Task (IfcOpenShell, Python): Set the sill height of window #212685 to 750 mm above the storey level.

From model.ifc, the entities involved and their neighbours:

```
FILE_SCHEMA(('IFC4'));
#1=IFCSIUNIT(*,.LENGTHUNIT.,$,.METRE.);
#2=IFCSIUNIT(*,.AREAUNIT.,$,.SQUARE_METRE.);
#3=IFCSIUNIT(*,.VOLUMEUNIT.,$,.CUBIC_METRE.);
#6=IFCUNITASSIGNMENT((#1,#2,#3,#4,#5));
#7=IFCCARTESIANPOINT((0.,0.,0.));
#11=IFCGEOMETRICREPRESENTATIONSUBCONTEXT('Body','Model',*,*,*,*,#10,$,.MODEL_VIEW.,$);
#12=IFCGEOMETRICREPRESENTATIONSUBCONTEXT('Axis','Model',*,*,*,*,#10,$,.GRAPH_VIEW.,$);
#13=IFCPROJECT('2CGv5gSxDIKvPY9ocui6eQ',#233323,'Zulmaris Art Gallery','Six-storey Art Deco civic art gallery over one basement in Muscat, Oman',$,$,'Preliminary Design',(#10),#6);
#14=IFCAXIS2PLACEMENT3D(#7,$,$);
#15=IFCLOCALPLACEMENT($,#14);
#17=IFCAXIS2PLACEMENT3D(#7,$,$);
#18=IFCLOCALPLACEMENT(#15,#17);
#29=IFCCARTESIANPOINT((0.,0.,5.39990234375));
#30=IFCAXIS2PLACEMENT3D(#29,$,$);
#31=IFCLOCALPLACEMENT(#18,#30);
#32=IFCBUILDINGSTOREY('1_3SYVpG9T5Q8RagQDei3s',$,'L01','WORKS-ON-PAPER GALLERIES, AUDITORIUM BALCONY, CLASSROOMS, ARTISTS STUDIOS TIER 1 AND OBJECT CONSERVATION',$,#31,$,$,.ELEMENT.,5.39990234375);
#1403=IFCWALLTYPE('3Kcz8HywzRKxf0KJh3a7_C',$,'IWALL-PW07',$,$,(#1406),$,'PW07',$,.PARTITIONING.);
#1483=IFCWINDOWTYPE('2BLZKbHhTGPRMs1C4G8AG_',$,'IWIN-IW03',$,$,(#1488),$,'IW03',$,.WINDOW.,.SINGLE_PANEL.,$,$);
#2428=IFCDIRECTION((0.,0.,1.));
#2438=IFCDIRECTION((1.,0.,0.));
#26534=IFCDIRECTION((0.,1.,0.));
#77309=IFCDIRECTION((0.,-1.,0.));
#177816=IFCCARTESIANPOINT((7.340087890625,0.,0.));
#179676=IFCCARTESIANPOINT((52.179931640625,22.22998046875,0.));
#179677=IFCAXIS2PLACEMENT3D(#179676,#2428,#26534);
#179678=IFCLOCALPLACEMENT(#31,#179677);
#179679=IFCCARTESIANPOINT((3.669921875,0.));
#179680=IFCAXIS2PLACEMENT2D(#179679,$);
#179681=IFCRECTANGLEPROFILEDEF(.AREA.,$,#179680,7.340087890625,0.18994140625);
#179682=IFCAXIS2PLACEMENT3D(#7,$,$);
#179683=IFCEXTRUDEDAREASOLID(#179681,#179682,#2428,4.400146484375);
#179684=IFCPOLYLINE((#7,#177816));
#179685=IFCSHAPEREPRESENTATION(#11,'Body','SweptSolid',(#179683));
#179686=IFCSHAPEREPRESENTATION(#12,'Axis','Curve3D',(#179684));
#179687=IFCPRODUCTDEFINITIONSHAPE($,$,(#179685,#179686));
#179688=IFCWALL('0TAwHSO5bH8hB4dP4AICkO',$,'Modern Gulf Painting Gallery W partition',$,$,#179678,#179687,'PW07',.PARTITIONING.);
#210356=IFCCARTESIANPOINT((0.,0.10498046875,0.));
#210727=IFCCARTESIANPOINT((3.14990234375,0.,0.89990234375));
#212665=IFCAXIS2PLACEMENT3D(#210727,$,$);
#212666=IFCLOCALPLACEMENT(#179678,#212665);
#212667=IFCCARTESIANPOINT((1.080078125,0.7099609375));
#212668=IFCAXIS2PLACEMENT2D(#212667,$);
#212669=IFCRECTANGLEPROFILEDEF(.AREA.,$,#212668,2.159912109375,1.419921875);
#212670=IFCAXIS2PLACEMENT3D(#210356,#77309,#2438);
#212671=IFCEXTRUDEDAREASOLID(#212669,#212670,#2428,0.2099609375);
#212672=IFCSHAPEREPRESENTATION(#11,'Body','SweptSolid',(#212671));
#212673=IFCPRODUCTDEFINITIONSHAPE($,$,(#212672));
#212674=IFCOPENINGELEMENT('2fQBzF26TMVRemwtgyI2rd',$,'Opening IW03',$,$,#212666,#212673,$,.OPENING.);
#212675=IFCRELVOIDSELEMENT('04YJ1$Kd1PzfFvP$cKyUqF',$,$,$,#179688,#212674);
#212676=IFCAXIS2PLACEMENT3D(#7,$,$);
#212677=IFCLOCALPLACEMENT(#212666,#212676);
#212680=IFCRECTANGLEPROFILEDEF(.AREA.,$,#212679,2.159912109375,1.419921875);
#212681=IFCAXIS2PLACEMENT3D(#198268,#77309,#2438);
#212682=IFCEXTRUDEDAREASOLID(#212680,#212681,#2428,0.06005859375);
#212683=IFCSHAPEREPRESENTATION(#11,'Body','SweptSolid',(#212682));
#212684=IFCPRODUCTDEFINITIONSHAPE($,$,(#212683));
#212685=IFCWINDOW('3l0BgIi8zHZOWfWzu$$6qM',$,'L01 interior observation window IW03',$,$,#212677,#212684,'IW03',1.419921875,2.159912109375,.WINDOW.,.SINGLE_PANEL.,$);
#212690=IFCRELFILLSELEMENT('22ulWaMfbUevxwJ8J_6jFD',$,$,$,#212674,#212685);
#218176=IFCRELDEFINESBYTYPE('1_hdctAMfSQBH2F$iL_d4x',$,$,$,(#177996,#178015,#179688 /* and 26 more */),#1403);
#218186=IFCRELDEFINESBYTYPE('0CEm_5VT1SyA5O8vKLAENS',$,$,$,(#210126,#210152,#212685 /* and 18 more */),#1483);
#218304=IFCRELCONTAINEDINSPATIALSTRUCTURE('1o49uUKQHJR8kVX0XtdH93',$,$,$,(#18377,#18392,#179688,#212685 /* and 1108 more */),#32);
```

```python
import numpy as np
import ifcopenshell
import ifcopenshell.api.geometry
import ifcopenshell.geom
import ifcopenshell.util.element
import ifcopenshell.util.placement
import ifcopenshell.util.shape
import ifcopenshell.util.unit

model = ifcopenshell.open("model.ifc")
unit_scale = ifcopenshell.util.unit.calculate_unit_scale(model)

window = model.by_id(212685)
opening = window.FillsVoids[0].RelatingOpeningElement
storey = ifcopenshell.util.element.get_container(window, ifc_class="IfcBuildingStorey")
level = ifcopenshell.util.placement.get_local_placement(storey.ObjectPlacement)[2, 3]

# The opening's origin need not be at the sill, so measure its lowest point.
shape = ifcopenshell.geom.create_shape(ifcopenshell.geom.settings(), opening)
bottom = ifcopenshell.util.shape.get_shape_bottom_elevation(shape, shape.geometry) / unit_scale
dz = level + 0.75 - bottom

shift = np.array([0.0, 0.0, dz])
# The window is placed relative to its opening, so it follows when the opening moves.
matrix = ifcopenshell.util.placement.get_local_placement(opening.ObjectPlacement)
matrix[:3, 3] += shift
ifcopenshell.api.geometry.edit_object_placement(
    model, product=opening, matrix=matrix, is_si=False, should_transform_children=True
)

print(f"moved by {dz * unit_scale:+.3f} m")

model.write("model_edited.ifc")
```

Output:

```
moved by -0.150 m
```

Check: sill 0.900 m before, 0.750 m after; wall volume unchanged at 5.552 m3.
